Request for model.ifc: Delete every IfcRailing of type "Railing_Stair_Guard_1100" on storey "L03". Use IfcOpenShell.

First a look at what the model holds.

```python
import ifcopenshell
import ifcopenshell.util.element

model = ifcopenshell.open("model.ifc")
print(model.schema)
storey = next(s for s in model.by_type("IfcBuildingStorey") if s.Name == "L03")
railings = [e for e in ifcopenshell.util.element.get_decomposition(storey) if e.is_a("IfcRailing")]
seen = {}
for e in railings:
    element_type = ifcopenshell.util.element.get_type(e)
    name = element_type.Name if element_type not in (None, e) else None
    seen[name] = seen.get(name, 0) + 1
for name, count in sorted(seen.items(), key=str):
    print(count, "x", name)
```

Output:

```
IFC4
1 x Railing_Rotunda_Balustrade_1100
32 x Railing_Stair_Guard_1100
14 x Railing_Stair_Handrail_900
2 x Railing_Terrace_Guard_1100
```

```python
import ifcopenshell
import ifcopenshell.api.root
import ifcopenshell.util.element

model = ifcopenshell.open("model.ifc")

storey = next(s for s in model.by_type("IfcBuildingStorey") if s.Name == "L03")
railings = [e for e in ifcopenshell.util.element.get_decomposition(storey) if e.is_a("IfcRailing")]
targets = [e for e in railings if (t := ifcopenshell.util.element.get_type(e)) not in (None, e) and t.Name == "Railing_Stair_Guard_1100"]

for e in targets:
    ifcopenshell.api.root.remove_product(model, product=e)
print(len(targets), "removed")

model.write("model_edited.ifc")
```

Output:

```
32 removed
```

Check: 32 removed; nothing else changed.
